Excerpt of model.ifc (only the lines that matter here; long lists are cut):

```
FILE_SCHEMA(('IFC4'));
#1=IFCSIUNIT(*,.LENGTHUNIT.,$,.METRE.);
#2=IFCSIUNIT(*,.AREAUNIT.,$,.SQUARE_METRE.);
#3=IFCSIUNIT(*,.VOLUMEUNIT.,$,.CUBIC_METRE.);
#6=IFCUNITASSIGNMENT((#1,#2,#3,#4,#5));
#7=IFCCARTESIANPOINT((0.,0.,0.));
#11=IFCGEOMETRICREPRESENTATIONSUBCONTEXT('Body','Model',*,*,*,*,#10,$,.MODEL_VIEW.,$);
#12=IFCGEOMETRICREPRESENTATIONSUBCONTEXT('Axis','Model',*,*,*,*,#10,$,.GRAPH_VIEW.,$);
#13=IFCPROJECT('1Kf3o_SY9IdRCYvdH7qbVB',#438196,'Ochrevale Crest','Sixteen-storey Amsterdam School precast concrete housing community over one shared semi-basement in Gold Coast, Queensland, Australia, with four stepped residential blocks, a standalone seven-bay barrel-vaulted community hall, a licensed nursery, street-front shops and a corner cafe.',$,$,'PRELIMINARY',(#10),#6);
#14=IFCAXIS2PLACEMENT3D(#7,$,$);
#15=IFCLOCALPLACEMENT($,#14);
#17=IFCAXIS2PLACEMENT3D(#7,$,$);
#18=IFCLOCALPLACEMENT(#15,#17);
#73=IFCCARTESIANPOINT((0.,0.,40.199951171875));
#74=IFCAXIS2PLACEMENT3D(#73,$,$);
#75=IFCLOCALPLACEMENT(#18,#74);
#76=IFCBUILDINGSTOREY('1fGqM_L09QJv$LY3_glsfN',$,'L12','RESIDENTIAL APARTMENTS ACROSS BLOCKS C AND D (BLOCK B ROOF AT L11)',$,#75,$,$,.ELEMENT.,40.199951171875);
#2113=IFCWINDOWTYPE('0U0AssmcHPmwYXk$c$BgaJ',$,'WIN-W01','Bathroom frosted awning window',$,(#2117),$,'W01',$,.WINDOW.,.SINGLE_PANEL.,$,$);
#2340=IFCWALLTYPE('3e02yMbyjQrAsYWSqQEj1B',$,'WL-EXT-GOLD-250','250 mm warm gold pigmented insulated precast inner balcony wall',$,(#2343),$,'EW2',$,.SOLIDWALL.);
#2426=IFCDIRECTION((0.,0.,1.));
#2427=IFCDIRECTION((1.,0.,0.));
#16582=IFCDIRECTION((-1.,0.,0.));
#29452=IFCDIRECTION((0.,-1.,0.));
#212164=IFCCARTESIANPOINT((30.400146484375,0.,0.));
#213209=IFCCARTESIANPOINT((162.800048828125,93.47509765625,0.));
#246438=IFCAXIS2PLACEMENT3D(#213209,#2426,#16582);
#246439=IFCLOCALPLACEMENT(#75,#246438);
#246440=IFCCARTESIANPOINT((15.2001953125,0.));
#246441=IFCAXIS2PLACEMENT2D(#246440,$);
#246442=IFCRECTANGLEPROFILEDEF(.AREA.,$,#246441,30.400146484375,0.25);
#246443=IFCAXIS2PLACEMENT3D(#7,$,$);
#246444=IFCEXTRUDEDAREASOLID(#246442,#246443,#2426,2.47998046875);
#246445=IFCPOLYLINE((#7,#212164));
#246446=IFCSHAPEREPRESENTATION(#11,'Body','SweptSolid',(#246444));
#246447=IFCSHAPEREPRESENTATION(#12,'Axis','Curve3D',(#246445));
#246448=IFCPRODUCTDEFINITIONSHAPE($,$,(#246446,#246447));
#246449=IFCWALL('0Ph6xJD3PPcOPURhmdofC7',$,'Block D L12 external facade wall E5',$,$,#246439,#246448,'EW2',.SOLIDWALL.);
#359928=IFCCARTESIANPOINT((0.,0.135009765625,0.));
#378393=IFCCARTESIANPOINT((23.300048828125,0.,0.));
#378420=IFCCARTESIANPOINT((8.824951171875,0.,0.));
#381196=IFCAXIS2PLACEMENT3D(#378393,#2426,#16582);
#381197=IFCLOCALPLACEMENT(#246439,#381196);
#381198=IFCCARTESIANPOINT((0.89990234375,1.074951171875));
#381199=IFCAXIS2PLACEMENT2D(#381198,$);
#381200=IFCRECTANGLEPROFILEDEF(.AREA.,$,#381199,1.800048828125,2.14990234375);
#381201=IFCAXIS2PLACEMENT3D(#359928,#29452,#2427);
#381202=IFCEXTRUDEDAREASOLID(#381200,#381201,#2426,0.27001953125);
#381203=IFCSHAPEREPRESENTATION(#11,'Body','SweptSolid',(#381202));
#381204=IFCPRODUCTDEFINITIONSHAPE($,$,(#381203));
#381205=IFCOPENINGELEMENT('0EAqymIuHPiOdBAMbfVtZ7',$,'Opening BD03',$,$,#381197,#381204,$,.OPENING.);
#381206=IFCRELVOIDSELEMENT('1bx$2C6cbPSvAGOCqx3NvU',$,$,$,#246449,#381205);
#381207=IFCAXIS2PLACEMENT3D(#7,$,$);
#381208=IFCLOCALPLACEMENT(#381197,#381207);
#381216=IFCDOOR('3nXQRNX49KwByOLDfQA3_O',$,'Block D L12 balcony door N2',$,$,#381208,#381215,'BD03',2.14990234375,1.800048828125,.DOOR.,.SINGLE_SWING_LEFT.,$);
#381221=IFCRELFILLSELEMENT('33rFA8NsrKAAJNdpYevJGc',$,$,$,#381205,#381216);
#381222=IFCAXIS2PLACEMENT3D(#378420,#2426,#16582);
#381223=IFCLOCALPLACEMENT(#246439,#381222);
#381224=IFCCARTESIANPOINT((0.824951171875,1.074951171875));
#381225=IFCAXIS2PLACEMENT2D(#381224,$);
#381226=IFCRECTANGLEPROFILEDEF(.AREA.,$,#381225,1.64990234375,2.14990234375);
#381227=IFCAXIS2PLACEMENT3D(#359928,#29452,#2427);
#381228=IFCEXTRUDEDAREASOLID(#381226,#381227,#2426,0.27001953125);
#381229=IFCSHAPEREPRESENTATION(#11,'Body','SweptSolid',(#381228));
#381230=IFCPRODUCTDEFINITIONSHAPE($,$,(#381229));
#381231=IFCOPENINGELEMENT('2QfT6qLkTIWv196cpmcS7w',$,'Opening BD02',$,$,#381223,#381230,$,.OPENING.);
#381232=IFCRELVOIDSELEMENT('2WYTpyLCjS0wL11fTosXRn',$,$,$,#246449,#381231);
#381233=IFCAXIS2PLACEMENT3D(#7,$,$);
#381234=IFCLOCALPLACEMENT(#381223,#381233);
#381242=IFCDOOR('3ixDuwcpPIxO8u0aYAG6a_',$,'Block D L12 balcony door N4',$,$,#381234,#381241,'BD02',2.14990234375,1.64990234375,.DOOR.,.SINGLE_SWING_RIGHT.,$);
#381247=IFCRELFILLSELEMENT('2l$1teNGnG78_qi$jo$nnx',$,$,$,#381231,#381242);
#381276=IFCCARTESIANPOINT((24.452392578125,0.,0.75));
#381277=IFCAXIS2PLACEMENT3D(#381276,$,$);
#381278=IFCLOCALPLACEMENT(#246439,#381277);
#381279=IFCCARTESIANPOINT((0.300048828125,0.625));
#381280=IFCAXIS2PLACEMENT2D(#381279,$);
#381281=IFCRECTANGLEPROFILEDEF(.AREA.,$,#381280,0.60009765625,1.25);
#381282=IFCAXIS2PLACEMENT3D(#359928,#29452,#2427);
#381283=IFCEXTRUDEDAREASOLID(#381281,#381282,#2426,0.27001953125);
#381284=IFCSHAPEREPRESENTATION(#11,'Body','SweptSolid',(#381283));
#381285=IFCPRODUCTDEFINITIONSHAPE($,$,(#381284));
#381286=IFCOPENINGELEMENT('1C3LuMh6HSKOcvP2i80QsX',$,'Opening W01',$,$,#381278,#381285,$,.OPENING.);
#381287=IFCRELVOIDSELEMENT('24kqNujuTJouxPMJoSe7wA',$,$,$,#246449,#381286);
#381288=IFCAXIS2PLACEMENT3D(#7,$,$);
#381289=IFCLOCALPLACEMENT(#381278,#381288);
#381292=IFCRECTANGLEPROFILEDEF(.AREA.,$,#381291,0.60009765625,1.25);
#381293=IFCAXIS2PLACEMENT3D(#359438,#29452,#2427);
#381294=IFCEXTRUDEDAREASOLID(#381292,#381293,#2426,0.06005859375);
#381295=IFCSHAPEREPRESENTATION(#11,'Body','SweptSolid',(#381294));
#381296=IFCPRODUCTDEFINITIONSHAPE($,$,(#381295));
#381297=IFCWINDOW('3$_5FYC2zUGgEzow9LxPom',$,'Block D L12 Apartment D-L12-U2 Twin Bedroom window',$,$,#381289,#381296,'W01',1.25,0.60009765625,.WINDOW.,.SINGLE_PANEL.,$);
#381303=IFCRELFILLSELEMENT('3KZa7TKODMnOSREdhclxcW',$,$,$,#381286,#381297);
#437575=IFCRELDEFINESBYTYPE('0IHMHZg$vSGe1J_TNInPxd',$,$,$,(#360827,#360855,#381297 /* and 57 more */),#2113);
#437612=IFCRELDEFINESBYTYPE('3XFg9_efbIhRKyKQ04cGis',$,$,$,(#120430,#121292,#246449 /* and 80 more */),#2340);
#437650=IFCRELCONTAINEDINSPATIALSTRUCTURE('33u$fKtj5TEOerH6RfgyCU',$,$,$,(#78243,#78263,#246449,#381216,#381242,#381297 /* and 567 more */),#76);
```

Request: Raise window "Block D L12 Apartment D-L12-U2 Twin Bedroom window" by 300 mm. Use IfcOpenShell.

```python
import numpy as np
import ifcopenshell
import ifcopenshell.api.geometry
import ifcopenshell.util.placement
import ifcopenshell.util.unit

model = ifcopenshell.open("model.ifc")
unit_scale = ifcopenshell.util.unit.calculate_unit_scale(model)

window = model.by_guid("3$_5FYC2zUGgEzow9LxPom")
opening = window.FillsVoids[0].RelatingOpeningElement
dz = 0.3 / unit_scale

shift = np.array([0.0, 0.0, dz])
# The window is placed relative to its opening, so it follows when the opening moves.
matrix = ifcopenshell.util.placement.get_local_placement(opening.ObjectPlacement)
matrix[:3, 3] += shift
ifcopenshell.api.geometry.edit_object_placement(
    model, product=opening, matrix=matrix, is_si=False, should_transform_children=True
)

print(f"moved by {dz * unit_scale:+.3f} m")

model.write("model_v2.ifc")
```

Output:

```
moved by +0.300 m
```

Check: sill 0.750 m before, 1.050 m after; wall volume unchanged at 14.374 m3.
